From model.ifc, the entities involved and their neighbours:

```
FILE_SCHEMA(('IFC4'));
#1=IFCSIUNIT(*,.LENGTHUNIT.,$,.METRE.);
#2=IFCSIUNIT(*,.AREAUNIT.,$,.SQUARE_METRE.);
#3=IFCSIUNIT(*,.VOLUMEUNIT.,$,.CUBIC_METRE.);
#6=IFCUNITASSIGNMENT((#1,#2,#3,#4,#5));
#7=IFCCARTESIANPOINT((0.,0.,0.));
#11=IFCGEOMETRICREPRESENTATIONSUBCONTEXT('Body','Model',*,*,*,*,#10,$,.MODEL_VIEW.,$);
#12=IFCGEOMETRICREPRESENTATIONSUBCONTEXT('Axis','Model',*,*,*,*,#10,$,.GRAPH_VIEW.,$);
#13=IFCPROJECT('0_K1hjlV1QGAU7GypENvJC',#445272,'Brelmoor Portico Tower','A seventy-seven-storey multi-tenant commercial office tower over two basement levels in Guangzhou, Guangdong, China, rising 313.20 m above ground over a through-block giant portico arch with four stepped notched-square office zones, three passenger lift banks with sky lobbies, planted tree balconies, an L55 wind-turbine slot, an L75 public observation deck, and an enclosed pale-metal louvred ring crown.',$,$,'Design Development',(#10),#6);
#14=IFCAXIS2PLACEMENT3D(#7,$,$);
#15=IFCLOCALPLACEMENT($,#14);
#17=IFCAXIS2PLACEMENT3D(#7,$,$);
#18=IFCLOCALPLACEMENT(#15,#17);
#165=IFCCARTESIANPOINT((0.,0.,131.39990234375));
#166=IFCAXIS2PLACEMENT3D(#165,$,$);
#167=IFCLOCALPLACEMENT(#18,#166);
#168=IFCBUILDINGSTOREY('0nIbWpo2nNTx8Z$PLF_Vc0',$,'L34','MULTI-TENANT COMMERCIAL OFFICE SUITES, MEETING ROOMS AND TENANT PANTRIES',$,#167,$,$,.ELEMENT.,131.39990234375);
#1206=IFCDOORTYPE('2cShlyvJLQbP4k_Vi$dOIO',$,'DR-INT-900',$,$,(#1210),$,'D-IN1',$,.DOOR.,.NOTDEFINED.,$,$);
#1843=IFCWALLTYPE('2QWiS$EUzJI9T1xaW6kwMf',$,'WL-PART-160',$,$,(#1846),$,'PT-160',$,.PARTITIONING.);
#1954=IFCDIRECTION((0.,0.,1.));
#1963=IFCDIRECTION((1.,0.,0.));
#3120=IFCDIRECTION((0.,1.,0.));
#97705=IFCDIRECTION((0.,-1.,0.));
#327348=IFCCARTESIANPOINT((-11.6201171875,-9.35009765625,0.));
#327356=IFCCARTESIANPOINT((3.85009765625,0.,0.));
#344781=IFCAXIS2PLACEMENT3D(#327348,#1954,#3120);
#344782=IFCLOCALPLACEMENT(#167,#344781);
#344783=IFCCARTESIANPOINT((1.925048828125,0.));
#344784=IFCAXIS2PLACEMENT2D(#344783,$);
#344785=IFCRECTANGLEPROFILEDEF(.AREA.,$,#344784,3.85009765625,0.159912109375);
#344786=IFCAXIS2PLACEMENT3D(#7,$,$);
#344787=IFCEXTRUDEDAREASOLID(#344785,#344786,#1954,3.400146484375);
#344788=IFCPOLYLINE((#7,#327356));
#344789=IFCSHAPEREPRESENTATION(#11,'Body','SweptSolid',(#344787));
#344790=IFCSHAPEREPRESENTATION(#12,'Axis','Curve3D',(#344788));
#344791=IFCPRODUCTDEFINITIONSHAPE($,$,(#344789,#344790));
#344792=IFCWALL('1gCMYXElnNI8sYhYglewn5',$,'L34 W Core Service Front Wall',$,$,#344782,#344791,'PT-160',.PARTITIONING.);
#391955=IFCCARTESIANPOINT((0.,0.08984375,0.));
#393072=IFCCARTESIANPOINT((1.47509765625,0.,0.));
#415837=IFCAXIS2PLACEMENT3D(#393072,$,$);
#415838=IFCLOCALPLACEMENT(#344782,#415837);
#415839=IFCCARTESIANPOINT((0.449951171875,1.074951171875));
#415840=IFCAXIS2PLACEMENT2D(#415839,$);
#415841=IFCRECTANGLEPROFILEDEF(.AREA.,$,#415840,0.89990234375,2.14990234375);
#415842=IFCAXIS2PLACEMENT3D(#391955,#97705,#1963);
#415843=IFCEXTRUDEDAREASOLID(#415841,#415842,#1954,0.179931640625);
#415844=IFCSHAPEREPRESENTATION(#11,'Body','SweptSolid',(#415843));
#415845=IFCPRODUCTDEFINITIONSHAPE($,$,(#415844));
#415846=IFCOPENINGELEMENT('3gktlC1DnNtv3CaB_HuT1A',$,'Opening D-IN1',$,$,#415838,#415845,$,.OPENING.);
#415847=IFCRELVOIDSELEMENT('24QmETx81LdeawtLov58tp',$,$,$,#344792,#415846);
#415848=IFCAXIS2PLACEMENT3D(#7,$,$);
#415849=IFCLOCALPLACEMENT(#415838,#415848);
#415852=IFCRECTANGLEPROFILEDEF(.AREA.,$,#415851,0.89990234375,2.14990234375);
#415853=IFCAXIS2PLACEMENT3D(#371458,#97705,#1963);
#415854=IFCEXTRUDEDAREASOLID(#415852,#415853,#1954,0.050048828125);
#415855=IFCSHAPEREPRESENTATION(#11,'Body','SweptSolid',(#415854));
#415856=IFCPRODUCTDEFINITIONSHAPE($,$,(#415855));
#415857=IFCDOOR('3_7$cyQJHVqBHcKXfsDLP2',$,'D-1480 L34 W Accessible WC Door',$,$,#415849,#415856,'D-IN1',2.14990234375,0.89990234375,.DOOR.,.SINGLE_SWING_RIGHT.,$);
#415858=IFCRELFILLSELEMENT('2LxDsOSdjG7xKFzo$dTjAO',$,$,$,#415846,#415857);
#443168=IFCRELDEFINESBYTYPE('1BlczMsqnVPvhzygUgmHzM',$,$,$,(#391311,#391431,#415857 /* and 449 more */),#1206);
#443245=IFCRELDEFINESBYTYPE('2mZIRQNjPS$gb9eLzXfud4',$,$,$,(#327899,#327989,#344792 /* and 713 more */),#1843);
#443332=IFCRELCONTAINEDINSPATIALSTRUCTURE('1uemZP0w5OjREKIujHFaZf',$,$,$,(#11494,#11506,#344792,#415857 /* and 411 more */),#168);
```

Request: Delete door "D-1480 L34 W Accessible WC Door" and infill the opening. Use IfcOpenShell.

```python
import ifcopenshell
import ifcopenshell.api.feature
import ifcopenshell.api.root
import ifcopenshell.geom
import ifcopenshell.util.shape

model = ifcopenshell.open("model.ifc")
settings = ifcopenshell.geom.settings()


def volume(element):
    """Net volume in cubic metres, openings subtracted."""
    shape = ifcopenshell.geom.create_shape(settings, element)
    return ifcopenshell.util.shape.get_volume(shape.geometry)


door = model.by_guid("3_7$cyQJHVqBHcKXfsDLP2")
opening = door.FillsVoids[0].RelatingOpeningElement
wall = opening.VoidsElements[0].RelatingBuildingElement
before = volume(wall)

ifcopenshell.api.root.remove_product(model, product=door)
ifcopenshell.api.feature.remove_feature(model, feature=opening)

after = volume(wall)

print(f"wall volume {before:.3f} -> {after:.3f} m3")

model.write("model-out.ifc")
```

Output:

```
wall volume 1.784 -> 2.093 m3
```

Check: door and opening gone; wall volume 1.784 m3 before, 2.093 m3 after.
